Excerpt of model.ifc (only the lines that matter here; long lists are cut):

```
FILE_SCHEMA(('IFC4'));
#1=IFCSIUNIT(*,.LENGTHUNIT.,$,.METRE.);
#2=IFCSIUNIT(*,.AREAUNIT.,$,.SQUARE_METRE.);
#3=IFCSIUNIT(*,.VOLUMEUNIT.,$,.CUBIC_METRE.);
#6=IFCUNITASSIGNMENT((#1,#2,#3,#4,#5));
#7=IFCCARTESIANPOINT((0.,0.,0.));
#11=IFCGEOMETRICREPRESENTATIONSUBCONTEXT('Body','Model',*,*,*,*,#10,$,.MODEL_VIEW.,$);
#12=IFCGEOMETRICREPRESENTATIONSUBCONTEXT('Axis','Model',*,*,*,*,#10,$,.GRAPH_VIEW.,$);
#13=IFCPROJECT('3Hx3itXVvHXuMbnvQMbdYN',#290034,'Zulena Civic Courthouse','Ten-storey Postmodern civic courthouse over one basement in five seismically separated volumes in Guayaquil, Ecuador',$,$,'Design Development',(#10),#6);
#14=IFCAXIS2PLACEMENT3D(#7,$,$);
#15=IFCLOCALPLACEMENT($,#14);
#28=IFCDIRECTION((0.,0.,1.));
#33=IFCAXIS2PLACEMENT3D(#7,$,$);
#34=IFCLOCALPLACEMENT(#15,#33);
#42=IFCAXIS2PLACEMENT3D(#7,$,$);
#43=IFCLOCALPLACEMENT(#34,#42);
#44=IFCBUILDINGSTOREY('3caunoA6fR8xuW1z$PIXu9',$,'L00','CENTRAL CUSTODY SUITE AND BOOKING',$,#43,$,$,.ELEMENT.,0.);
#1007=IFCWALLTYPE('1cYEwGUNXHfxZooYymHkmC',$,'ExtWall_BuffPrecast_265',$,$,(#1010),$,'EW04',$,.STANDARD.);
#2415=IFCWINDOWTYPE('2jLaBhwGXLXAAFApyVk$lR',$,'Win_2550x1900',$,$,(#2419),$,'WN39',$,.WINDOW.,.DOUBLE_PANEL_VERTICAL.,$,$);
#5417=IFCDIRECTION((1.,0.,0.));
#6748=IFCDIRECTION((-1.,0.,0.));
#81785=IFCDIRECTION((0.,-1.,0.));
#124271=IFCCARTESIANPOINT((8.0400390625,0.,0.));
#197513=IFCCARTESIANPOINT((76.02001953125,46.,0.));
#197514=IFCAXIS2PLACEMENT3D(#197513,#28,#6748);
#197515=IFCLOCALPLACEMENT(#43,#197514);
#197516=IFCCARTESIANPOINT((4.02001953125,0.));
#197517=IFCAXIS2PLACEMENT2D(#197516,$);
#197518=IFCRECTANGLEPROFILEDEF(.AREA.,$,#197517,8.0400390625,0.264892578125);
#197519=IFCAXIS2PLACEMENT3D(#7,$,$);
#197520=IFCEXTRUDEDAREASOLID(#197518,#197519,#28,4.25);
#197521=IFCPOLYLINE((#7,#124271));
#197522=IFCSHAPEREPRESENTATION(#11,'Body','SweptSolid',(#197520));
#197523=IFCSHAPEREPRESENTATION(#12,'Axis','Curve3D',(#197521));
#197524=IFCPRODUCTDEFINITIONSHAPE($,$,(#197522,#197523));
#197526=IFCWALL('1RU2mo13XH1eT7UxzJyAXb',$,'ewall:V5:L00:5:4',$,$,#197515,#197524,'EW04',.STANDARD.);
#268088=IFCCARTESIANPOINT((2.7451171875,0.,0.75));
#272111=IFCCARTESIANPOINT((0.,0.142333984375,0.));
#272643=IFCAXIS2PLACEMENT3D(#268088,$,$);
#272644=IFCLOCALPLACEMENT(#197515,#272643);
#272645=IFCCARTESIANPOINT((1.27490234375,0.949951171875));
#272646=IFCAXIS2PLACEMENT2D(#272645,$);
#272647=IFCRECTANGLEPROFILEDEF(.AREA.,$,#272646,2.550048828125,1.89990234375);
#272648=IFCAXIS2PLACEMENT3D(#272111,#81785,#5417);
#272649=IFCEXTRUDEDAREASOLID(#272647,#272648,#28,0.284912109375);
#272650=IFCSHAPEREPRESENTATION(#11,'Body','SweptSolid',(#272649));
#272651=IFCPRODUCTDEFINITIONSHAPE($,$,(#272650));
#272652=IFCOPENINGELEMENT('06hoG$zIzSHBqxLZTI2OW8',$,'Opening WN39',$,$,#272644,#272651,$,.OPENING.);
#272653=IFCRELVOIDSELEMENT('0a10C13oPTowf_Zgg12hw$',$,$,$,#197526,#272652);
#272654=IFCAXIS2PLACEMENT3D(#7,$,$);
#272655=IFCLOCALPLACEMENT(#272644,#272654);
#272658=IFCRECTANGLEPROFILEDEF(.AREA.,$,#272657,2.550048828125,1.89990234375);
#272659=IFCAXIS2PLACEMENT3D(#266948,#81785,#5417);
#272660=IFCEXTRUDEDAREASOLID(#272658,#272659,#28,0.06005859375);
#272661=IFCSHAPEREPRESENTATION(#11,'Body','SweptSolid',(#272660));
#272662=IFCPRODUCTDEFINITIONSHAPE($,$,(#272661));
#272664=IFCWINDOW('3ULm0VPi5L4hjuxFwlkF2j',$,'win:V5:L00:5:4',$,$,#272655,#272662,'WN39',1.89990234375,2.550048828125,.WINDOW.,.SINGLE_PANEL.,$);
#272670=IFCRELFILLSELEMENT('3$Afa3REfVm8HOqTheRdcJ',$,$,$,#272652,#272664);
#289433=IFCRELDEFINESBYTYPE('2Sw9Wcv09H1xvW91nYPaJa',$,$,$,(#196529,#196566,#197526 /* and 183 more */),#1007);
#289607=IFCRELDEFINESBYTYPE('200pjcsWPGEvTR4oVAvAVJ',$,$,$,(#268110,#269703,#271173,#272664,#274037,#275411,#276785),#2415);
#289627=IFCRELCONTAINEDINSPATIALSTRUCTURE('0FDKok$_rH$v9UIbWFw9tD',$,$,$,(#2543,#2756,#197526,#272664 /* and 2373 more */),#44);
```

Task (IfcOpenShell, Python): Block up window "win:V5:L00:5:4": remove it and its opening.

```python
import ifcopenshell
import ifcopenshell.api.feature
import ifcopenshell.api.root
import ifcopenshell.geom
import ifcopenshell.util.shape

model = ifcopenshell.open("model.ifc")
settings = ifcopenshell.geom.settings()


def volume(element):
    """Net volume in cubic metres, openings subtracted."""
    shape = ifcopenshell.geom.create_shape(settings, element)
    return ifcopenshell.util.shape.get_volume(shape.geometry)


window = model.by_guid("3ULm0VPi5L4hjuxFwlkF2j")
opening = window.FillsVoids[0].RelatingOpeningElement
wall = opening.VoidsElements[0].RelatingBuildingElement
before = volume(wall)

ifcopenshell.api.root.remove_product(model, product=window)
ifcopenshell.api.feature.remove_feature(model, feature=opening)

after = volume(wall)

print(f"wall volume {before:.3f} -> {after:.3f} m3")

model.write("model_updated.ifc")
```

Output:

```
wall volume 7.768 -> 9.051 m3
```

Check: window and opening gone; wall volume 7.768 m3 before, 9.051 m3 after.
